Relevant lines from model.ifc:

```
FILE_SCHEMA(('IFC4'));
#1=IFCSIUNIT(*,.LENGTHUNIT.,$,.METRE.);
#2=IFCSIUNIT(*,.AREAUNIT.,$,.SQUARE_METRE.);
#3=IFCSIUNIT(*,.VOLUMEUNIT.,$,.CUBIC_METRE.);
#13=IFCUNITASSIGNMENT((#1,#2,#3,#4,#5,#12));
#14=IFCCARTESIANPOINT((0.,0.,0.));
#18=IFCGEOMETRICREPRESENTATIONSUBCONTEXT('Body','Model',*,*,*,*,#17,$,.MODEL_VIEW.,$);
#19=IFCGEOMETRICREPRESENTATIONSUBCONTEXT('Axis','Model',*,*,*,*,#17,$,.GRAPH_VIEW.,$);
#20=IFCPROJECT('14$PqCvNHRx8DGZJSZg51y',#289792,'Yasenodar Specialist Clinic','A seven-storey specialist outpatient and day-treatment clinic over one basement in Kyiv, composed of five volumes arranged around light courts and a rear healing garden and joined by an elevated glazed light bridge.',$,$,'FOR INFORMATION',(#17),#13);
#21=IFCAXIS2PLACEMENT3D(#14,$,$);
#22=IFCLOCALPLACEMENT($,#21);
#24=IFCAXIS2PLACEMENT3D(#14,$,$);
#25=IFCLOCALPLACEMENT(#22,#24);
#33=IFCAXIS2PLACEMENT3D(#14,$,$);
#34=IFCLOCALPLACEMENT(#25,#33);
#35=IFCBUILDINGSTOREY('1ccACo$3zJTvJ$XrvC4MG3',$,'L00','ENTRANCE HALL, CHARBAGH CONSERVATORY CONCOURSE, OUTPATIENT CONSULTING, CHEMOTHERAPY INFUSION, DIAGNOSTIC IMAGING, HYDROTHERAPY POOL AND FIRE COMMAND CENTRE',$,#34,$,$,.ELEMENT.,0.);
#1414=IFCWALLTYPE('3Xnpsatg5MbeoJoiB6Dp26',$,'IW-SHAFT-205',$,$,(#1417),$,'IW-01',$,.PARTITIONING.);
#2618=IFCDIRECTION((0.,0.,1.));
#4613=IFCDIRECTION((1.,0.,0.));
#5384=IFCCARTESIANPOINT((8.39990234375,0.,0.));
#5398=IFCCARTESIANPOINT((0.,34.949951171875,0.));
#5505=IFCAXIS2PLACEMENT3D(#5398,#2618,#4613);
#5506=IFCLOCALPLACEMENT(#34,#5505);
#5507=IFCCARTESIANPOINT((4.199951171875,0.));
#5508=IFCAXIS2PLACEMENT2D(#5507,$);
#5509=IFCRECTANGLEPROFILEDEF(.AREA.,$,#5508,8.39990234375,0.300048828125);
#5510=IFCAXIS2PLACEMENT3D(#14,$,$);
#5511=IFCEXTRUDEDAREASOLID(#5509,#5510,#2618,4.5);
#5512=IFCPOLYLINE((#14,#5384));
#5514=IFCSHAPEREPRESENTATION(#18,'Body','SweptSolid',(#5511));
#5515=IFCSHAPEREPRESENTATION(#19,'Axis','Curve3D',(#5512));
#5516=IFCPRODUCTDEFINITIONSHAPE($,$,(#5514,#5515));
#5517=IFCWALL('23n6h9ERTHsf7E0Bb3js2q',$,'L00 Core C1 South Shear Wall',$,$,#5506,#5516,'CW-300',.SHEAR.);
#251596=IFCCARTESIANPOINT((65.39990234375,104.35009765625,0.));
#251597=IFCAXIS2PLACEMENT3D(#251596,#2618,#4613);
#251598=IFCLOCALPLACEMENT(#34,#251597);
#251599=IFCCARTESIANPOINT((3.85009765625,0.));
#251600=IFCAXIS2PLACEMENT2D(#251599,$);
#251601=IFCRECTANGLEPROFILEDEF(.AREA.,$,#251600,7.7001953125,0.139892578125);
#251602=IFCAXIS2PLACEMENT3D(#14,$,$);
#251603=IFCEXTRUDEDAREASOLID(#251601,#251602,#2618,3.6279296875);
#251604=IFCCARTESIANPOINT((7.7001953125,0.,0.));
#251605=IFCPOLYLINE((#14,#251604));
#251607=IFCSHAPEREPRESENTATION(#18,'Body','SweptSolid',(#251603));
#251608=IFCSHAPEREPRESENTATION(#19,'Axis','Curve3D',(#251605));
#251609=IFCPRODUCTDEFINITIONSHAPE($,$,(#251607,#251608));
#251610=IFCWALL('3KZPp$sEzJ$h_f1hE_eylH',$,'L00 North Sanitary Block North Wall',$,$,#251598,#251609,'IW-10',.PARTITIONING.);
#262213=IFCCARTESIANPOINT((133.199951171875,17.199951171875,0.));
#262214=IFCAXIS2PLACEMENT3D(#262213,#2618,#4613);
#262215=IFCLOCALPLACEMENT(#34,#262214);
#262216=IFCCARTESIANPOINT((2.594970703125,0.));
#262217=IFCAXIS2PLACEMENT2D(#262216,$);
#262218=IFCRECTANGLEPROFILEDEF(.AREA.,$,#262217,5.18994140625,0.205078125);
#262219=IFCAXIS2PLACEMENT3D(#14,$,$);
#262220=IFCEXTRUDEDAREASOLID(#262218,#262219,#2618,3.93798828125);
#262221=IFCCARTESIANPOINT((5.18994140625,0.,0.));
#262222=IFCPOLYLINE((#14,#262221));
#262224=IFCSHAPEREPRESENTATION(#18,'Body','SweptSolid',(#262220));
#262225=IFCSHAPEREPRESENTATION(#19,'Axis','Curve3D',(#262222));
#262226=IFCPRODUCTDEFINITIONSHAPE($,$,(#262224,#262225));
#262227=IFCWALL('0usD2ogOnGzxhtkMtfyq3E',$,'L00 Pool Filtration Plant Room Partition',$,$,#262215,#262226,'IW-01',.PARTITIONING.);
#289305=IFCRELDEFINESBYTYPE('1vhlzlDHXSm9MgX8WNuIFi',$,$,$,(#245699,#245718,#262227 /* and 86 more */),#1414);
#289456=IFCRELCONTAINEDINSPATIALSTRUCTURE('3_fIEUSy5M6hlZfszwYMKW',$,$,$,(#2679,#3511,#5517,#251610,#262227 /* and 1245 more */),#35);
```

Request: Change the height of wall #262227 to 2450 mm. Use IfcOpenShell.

```python
import ifcopenshell
import ifcopenshell.geom
import ifcopenshell.util.representation
import ifcopenshell.util.shape
import ifcopenshell.util.unit

model = ifcopenshell.open("model.ifc")
unit_scale = ifcopenshell.util.unit.calculate_unit_scale(model)
settings = ifcopenshell.geom.settings()


def volume(element):
    """Net volume in cubic metres, openings subtracted."""
    shape = ifcopenshell.geom.create_shape(settings, element)
    return ifcopenshell.util.shape.get_volume(shape.geometry)


wall = model.by_id(262227)
before = volume(wall)

body = ifcopenshell.util.representation.get_representation(wall, "Model", "Body")
solid = body.Items[0]
old_height = solid.Depth
solid.Depth = 2.45 / unit_scale
after = volume(wall)

print(f"height {old_height:g} -> {solid.Depth:g}, volume {before:.3f} -> {after:.3f} m3")

model.write("model_edited.ifc")
```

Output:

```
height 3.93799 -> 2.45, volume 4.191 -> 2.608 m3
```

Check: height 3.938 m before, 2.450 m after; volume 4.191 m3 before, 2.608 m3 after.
